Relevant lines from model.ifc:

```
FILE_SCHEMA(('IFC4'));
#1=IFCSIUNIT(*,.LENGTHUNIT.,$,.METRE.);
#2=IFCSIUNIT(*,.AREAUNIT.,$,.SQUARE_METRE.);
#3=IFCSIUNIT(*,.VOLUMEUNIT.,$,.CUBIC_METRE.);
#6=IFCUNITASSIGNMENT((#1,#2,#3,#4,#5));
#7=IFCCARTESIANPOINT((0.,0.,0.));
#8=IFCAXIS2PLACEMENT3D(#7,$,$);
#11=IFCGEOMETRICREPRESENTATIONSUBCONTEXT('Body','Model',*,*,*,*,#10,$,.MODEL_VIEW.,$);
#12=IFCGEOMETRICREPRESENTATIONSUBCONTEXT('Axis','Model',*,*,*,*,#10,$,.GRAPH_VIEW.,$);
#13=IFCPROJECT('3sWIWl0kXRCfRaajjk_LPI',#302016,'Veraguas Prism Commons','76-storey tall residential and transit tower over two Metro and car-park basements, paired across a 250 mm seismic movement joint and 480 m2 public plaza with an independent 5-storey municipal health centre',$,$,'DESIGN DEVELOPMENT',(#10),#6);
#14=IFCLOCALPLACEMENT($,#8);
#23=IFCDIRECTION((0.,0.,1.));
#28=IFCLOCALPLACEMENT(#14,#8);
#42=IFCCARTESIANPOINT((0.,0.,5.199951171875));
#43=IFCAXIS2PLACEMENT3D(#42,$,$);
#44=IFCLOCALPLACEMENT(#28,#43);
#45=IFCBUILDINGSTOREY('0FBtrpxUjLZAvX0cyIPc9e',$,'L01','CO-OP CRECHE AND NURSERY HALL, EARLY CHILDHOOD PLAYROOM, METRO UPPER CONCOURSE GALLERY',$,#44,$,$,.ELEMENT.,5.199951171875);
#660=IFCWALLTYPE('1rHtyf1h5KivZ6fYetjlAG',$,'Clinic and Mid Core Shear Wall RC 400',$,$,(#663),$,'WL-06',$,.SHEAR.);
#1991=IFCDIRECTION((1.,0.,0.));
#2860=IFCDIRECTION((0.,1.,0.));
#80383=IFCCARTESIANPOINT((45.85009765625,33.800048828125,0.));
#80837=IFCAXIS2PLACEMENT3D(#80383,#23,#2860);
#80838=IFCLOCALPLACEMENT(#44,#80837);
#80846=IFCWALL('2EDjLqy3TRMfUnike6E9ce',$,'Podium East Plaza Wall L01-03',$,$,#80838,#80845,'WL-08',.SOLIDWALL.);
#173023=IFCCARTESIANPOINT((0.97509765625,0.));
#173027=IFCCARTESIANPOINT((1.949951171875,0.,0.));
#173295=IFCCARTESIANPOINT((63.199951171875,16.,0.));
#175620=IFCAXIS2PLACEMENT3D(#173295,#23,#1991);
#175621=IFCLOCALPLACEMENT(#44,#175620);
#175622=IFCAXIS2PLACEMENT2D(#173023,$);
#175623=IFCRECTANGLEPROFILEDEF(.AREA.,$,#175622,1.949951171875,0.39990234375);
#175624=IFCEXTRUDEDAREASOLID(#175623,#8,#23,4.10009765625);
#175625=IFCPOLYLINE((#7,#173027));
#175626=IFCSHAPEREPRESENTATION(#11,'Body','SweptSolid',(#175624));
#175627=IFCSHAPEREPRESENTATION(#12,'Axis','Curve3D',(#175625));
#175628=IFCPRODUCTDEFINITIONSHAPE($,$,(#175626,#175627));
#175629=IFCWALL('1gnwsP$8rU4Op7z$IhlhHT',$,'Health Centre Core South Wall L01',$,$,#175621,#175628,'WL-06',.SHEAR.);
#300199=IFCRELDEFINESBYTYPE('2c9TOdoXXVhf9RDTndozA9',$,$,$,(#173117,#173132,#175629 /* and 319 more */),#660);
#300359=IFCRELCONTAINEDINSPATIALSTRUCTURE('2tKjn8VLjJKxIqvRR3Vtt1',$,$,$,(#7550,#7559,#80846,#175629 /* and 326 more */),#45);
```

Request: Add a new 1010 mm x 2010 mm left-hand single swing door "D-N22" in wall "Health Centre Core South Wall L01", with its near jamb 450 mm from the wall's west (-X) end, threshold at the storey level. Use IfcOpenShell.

```python
import numpy as np
import ifcopenshell
import ifcopenshell.api.feature
import ifcopenshell.api.geometry
import ifcopenshell.api.root
import ifcopenshell.api.spatial
import ifcopenshell.geom
import ifcopenshell.util.element
import ifcopenshell.util.placement
import ifcopenshell.util.representation
import ifcopenshell.util.shape
import ifcopenshell.util.unit

model = ifcopenshell.open("model.ifc")
unit_scale = ifcopenshell.util.unit.calculate_unit_scale(model)
settings = ifcopenshell.geom.settings()


def volume(element):
    """Net volume in cubic metres, openings subtracted."""
    shape = ifcopenshell.geom.create_shape(settings, element)
    return ifcopenshell.util.shape.get_volume(shape.geometry)


wall = model.by_guid("1gnwsP$8rU4Op7z$IhlhHT")
storey = ifcopenshell.util.element.get_container(wall, ifc_class="IfcBuildingStorey")
context = ifcopenshell.util.representation.get_context(model, "Model", "Body", "MODEL_VIEW")
before = volume(wall)

width, height, from_end, sill = 1.01, 2.01, 0.45, 0.0  # metres

# The wall runs along its own X axis, and the end named is its -X end.
wall_shape = ifcopenshell.geom.create_shape(settings, wall)
x, y, z = ifcopenshell.util.shape.get_vertices(wall_shape.geometry).T
start = x.min() + from_end
face, thickness = float(y.min()), float(y.max() - y.min())
wall_matrix = ifcopenshell.util.placement.get_local_placement(wall.ObjectPlacement)
level = ifcopenshell.util.placement.get_local_placement(storey.ObjectPlacement)[2, 3]


def in_wall(x, y):
    """Placement at x, y metres in the wall's axes, at sill height."""
    matrix = wall_matrix.copy()
    matrix[:, 3] = wall_matrix @ np.array([x / unit_scale, y / unit_scale, 0.0, 1.0])
    matrix[2, 3] = level + sill / unit_scale
    return matrix


# Opening: a box that overshoots both wall faces by 50 mm.
opening = ifcopenshell.api.root.create_entity(model, ifc_class="IfcOpeningElement", predefined_type="OPENING")
box = ifcopenshell.api.geometry.add_wall_representation(
    model, context=context, length=width, height=height, thickness=thickness + 0.1
)
ifcopenshell.api.geometry.assign_representation(model, product=opening, representation=box)
ifcopenshell.api.geometry.edit_object_placement(model, product=opening, matrix=in_wall(start, face - 0.05), is_si=False)
ifcopenshell.api.feature.add_feature(model, feature=opening, element=wall)

door = ifcopenshell.api.root.create_entity(model, ifc_class="IfcDoor", name="D-N22", predefined_type="DOOR")
door.OverallWidth, door.OverallHeight = width / unit_scale, height / unit_scale
door.OperationType = "SINGLE_SWING_LEFT"
body = ifcopenshell.api.geometry.add_door_representation(
    model,
    context=context,
    overall_width=door.OverallWidth,
    overall_height=door.OverallHeight,
    operation_type="SINGLE_SWING_LEFT",
    lining_properties={"LiningDepth": thickness / unit_scale, "ThresholdDepth": thickness / unit_scale},
)
ifcopenshell.api.geometry.assign_representation(model, product=door, representation=body)
ifcopenshell.api.spatial.assign_container(model, products=[door], relating_structure=storey)
ifcopenshell.api.feature.add_filling(model, opening=opening, element=door)

# The lining spans the wall, so the door starts at the wall face.
ifcopenshell.api.geometry.edit_object_placement(model, product=door, matrix=in_wall(start, face), is_si=False)

after = volume(wall)

print(f"wall volume {before:.3f} -> {after:.3f} m3")

model.write("model_rev.ifc")
```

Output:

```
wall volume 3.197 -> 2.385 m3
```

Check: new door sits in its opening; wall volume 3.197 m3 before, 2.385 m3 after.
